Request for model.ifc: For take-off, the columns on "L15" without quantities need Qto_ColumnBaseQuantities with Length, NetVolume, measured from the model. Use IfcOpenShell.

First a look at what the model holds.

```python
import ifcopenshell
import ifcopenshell.util.element
import ifcopenshell.util.unit

model = ifcopenshell.open("model.ifc")
print(model.schema)
for unit_type in ("LENGTHUNIT", "AREAUNIT", "VOLUMEUNIT"):
    print(unit_type, ifcopenshell.util.unit.calculate_unit_scale(model, unit_type))
storey = next(s for s in model.by_type("IfcBuildingStorey") if s.Name == "L15")
columns = [e for e in ifcopenshell.util.element.get_decomposition(storey) if e.is_a("IfcColumn")]
for e in sorted(columns, key=lambda e: e.id()):
    print(e.id(), e.is_a(), e.Name, list(ifcopenshell.util.element.get_psets(e, qtos_only=True)), sep=" | ")
```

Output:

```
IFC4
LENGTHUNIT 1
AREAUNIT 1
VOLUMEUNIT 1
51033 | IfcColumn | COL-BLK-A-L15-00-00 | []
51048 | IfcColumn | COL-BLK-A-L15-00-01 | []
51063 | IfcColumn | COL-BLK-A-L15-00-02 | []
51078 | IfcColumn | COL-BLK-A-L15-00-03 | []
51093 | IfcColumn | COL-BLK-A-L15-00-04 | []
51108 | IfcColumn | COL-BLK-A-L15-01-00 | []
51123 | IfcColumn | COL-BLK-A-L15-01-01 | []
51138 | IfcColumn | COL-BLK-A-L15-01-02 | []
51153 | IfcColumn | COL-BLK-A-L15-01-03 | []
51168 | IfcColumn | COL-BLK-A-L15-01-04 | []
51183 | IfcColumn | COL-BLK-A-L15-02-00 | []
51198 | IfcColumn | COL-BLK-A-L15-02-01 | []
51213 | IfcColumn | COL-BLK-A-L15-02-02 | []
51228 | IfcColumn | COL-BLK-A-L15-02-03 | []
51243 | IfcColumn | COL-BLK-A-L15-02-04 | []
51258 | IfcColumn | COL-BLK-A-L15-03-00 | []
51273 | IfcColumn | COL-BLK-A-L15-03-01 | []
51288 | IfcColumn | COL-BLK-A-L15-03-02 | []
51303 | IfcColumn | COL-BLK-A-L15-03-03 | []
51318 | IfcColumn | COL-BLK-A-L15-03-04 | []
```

```python
import ifcopenshell
import ifcopenshell.api.pset
import ifcopenshell.geom
import ifcopenshell.util.element
import ifcopenshell.util.shape
import ifcopenshell.util.unit

model = ifcopenshell.open("model.ifc")
unit_scale = ifcopenshell.util.unit.calculate_unit_scale(model)
volume_scale = ifcopenshell.util.unit.calculate_unit_scale(model, "VOLUMEUNIT")
settings = ifcopenshell.geom.settings()

storey = next(s for s in model.by_type("IfcBuildingStorey") if s.Name == "L15")
columns = [e for e in ifcopenshell.util.element.get_decomposition(storey) if e.is_a("IfcColumn")]

for e in sorted(columns, key=lambda e: e.id()):
    if ifcopenshell.util.element.get_psets(e, qtos_only=True, should_inherit=False):
        continue
    # Geometry comes back in metres, in the element's own axes.
    shape = ifcopenshell.geom.create_shape(settings, e)
    values = {
        "Length": ifcopenshell.util.shape.get_z(shape.geometry) / unit_scale,
        "NetVolume": ifcopenshell.util.shape.get_volume(shape.geometry) / volume_scale,
    }
    qto = ifcopenshell.api.pset.add_qto(model, product=e, name="Qto_ColumnBaseQuantities")
    ifcopenshell.api.pset.edit_qto(model, qto=qto, properties=values)
    print(e.id(), {k: round(v, 3) for k, v in values.items()})

model.write("model_updated.ifc")
```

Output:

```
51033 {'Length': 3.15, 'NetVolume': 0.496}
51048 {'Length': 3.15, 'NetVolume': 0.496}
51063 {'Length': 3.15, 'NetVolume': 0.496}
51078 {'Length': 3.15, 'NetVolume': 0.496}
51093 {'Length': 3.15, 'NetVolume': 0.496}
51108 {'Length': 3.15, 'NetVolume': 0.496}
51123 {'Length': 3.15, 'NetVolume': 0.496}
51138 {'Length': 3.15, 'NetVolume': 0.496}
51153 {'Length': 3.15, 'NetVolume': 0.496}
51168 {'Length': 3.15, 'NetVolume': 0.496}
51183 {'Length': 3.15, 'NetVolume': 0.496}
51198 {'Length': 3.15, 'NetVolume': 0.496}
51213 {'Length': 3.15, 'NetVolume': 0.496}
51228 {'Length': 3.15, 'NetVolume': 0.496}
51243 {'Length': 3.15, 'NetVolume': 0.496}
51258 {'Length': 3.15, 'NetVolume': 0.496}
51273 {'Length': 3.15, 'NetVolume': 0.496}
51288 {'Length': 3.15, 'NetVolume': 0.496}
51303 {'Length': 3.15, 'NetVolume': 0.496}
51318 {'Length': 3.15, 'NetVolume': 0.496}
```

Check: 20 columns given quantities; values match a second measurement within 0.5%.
